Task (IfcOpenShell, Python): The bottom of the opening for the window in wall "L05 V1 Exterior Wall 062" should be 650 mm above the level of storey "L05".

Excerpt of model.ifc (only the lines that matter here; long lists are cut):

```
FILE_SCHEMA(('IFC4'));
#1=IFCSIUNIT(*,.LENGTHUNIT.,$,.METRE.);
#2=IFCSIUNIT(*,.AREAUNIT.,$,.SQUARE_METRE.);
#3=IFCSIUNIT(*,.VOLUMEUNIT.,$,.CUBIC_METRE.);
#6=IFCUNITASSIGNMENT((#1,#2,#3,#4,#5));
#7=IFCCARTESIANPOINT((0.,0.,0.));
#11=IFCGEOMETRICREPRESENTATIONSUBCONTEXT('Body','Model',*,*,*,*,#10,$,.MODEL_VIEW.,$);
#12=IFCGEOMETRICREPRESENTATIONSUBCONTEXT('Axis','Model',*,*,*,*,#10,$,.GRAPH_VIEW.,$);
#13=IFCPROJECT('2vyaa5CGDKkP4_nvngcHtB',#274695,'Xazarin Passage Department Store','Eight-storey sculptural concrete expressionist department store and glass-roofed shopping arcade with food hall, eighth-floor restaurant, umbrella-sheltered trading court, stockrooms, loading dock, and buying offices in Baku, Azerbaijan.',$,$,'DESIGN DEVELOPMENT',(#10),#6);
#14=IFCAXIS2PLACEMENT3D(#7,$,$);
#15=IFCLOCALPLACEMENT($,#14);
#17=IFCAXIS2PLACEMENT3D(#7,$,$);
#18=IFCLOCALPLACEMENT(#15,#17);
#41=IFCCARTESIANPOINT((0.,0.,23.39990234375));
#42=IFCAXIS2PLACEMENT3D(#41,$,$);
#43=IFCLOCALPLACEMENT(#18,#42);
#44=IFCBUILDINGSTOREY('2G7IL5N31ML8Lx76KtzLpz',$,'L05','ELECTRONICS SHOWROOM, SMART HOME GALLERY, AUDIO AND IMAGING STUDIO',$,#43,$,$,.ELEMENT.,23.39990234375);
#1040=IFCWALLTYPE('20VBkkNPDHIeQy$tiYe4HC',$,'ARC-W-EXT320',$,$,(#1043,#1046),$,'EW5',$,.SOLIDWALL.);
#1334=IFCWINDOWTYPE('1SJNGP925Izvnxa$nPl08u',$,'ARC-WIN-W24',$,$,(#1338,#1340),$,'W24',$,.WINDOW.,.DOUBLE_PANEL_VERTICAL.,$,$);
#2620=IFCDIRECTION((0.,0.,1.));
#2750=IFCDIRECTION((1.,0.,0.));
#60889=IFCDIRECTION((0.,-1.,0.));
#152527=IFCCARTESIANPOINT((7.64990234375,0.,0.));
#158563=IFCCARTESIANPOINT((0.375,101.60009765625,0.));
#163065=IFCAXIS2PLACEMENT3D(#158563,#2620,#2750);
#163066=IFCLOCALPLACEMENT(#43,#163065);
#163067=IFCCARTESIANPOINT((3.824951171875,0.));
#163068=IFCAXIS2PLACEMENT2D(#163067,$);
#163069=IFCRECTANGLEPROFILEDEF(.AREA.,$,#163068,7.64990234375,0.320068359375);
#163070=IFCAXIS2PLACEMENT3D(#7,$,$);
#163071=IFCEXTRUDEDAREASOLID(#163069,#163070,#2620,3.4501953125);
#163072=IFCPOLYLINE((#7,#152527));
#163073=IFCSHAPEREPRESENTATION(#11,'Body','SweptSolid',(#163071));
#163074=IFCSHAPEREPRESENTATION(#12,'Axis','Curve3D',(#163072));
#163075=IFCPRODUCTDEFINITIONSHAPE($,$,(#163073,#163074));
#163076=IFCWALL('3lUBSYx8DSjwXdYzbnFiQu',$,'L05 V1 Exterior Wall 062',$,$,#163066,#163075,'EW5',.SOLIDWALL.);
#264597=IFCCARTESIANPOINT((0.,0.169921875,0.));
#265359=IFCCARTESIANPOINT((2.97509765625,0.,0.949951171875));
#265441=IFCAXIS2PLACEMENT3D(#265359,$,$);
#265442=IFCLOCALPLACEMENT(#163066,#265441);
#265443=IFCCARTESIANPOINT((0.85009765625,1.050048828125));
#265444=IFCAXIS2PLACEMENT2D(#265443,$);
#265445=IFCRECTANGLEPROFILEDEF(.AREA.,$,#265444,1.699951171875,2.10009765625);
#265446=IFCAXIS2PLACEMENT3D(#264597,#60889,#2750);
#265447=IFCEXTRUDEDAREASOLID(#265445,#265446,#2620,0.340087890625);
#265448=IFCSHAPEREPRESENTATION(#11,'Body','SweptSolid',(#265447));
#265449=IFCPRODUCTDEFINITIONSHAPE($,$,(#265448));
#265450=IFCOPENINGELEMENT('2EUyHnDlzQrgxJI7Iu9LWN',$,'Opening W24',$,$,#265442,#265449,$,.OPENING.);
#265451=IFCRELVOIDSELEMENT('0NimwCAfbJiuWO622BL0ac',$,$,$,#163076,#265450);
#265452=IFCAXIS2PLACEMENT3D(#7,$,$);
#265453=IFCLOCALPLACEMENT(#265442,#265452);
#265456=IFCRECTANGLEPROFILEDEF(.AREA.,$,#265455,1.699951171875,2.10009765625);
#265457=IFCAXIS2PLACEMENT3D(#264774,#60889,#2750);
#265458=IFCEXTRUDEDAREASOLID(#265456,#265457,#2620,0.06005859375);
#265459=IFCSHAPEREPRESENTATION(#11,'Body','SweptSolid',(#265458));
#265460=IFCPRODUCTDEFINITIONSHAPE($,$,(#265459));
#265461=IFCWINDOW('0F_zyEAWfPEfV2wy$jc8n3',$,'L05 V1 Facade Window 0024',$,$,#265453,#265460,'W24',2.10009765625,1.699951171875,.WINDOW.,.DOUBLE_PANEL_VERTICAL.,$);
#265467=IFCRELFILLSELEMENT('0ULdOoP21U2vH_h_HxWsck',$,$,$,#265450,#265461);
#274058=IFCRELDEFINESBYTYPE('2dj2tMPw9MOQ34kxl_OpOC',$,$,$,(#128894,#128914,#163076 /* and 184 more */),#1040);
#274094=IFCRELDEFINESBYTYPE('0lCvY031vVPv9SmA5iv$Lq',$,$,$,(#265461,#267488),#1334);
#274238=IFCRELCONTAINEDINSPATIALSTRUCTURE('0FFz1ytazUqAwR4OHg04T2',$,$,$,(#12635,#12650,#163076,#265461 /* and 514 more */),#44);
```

```python
import numpy as np
import ifcopenshell
import ifcopenshell.api.geometry
import ifcopenshell.geom
import ifcopenshell.util.element
import ifcopenshell.util.placement
import ifcopenshell.util.shape
import ifcopenshell.util.unit

model = ifcopenshell.open("model.ifc")
unit_scale = ifcopenshell.util.unit.calculate_unit_scale(model)

window = model.by_guid("0F_zyEAWfPEfV2wy$jc8n3")
opening = window.FillsVoids[0].RelatingOpeningElement
storey = ifcopenshell.util.element.get_container(window, ifc_class="IfcBuildingStorey")
level = ifcopenshell.util.placement.get_local_placement(storey.ObjectPlacement)[2, 3]

# The opening's origin need not be at the sill, so measure its lowest point.
shape = ifcopenshell.geom.create_shape(ifcopenshell.geom.settings(), opening)
bottom = ifcopenshell.util.shape.get_shape_bottom_elevation(shape, shape.geometry) / unit_scale
dz = level + 0.65 / unit_scale - bottom

shift = np.array([0.0, 0.0, dz])
# The window is placed relative to its opening, so it follows when the opening moves.
matrix = ifcopenshell.util.placement.get_local_placement(opening.ObjectPlacement)
matrix[:3, 3] += shift
ifcopenshell.api.geometry.edit_object_placement(
    model, product=opening, matrix=matrix, is_si=False, should_transform_children=True
)

print(f"moved by {dz * unit_scale:+.3f} m")

model.write("model_updated.ifc")
```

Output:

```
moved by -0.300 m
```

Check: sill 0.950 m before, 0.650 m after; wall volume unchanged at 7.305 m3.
